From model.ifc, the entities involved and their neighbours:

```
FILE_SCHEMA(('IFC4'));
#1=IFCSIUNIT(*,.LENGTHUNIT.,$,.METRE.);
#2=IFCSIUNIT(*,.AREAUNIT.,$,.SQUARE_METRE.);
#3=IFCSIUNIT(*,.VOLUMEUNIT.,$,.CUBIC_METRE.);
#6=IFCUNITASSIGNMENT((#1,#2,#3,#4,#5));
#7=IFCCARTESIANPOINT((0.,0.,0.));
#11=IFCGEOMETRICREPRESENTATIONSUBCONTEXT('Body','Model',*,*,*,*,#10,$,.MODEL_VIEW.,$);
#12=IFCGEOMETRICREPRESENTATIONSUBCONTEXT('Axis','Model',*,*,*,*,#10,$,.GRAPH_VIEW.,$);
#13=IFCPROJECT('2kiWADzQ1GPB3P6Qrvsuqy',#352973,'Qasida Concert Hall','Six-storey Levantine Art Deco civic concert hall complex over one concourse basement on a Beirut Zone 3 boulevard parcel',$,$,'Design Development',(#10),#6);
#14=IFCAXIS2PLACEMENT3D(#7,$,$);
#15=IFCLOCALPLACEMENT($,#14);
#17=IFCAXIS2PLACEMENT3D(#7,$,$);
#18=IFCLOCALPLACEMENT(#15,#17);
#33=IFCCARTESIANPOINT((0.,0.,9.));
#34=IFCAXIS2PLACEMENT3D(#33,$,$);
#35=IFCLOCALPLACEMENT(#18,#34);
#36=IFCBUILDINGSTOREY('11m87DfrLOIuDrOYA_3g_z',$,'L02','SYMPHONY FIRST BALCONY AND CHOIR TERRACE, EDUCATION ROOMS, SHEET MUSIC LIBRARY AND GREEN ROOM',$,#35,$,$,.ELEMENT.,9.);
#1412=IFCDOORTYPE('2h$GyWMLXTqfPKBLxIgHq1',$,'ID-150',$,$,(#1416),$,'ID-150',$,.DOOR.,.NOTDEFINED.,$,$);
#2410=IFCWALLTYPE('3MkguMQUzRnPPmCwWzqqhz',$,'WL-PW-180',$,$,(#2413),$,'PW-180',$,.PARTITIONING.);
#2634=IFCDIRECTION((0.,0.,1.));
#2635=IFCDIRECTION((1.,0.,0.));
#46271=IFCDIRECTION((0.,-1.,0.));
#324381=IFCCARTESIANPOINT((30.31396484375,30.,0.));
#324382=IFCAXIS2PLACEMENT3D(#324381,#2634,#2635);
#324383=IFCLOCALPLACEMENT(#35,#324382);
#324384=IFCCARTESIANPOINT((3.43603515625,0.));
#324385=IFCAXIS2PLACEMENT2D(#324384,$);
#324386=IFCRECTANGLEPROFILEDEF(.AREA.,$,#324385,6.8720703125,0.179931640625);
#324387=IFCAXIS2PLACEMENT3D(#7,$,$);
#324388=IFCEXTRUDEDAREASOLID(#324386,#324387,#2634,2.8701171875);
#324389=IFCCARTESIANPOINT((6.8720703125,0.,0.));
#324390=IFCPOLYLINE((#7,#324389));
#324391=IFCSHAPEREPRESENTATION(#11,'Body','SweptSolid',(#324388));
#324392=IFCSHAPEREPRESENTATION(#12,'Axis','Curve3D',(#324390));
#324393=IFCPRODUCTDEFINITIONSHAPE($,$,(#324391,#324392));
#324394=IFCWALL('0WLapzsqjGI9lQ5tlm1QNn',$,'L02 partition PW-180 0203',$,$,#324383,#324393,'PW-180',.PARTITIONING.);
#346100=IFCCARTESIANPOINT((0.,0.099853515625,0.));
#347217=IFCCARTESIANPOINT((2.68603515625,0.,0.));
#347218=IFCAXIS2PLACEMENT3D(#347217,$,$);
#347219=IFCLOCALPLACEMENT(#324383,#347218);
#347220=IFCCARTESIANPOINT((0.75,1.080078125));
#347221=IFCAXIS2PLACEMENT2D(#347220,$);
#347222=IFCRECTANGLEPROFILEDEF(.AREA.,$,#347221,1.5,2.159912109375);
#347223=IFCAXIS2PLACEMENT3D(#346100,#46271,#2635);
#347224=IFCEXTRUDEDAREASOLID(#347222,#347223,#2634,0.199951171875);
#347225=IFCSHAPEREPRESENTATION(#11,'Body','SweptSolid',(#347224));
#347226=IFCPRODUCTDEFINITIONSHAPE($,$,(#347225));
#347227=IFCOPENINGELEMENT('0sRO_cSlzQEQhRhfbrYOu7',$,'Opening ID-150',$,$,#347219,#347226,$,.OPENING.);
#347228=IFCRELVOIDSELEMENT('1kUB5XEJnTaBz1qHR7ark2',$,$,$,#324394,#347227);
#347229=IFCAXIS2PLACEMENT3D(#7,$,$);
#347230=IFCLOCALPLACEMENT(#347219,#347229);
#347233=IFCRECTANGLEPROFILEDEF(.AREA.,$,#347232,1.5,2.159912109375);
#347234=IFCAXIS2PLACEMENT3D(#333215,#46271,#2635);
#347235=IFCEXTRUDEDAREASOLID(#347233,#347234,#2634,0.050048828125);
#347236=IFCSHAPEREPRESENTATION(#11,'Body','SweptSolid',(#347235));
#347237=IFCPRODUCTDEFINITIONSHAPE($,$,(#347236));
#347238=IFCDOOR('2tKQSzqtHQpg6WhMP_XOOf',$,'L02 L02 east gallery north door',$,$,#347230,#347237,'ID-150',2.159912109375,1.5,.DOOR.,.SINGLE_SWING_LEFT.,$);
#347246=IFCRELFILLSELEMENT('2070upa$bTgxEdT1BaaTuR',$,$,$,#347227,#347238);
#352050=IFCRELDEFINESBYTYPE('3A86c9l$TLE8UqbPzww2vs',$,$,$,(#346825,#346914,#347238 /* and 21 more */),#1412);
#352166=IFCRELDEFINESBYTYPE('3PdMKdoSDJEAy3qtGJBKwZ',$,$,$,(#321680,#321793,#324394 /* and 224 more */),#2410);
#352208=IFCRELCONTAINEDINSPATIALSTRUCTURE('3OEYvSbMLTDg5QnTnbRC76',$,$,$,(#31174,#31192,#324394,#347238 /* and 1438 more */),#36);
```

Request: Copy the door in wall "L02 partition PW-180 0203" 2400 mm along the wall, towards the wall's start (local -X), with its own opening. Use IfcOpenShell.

```python
import ifcopenshell
import ifcopenshell.api.feature
import ifcopenshell.api.geometry
import ifcopenshell.api.root
import ifcopenshell.geom
import ifcopenshell.util.element
import ifcopenshell.util.placement
import ifcopenshell.util.shape

model = ifcopenshell.open("model.ifc")
settings = ifcopenshell.geom.settings()


def volume(element):
    """Net volume in cubic metres, openings subtracted."""
    shape = ifcopenshell.geom.create_shape(settings, element)
    return ifcopenshell.util.shape.get_volume(shape.geometry)


door = model.by_guid("2tKQSzqtHQpg6WhMP_XOOf")
opening = door.FillsVoids[0].RelatingOpeningElement
wall = opening.VoidsElements[0].RelatingBuildingElement
before = volume(wall)
shift = ifcopenshell.util.placement.get_local_placement(wall.ObjectPlacement)[:3, 0] * -2.4

# copy_class copies the void relationship, type, container and properties, but no geometry.
new_opening = ifcopenshell.api.root.copy_class(model, product=opening)
new_opening.Representation = ifcopenshell.util.element.copy_deep(
    model, opening.Representation, exclude=["IfcGeometricRepresentationContext", "IfcRepresentationMap"]
)
new_door = ifcopenshell.api.root.copy_class(model, product=door)
new_door.Representation = ifcopenshell.util.element.copy_deep(
    model, door.Representation, exclude=["IfcGeometricRepresentationContext", "IfcRepresentationMap"]
)
new_door.Tag = None
ifcopenshell.api.feature.add_filling(model, opening=new_opening, element=new_door)

for old, new in ((opening, new_opening), (door, new_door)):
    matrix = ifcopenshell.util.placement.get_local_placement(old.ObjectPlacement)
    matrix[:3, 3] += shift
    ifcopenshell.api.geometry.edit_object_placement(model, product=new, matrix=matrix, is_si=False)

after = volume(wall)

print(f"wall volume {before:.3f} -> {after:.3f} m3")

model.write("model-out.ifc")
```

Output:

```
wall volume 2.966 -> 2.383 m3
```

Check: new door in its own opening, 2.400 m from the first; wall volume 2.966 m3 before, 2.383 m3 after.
